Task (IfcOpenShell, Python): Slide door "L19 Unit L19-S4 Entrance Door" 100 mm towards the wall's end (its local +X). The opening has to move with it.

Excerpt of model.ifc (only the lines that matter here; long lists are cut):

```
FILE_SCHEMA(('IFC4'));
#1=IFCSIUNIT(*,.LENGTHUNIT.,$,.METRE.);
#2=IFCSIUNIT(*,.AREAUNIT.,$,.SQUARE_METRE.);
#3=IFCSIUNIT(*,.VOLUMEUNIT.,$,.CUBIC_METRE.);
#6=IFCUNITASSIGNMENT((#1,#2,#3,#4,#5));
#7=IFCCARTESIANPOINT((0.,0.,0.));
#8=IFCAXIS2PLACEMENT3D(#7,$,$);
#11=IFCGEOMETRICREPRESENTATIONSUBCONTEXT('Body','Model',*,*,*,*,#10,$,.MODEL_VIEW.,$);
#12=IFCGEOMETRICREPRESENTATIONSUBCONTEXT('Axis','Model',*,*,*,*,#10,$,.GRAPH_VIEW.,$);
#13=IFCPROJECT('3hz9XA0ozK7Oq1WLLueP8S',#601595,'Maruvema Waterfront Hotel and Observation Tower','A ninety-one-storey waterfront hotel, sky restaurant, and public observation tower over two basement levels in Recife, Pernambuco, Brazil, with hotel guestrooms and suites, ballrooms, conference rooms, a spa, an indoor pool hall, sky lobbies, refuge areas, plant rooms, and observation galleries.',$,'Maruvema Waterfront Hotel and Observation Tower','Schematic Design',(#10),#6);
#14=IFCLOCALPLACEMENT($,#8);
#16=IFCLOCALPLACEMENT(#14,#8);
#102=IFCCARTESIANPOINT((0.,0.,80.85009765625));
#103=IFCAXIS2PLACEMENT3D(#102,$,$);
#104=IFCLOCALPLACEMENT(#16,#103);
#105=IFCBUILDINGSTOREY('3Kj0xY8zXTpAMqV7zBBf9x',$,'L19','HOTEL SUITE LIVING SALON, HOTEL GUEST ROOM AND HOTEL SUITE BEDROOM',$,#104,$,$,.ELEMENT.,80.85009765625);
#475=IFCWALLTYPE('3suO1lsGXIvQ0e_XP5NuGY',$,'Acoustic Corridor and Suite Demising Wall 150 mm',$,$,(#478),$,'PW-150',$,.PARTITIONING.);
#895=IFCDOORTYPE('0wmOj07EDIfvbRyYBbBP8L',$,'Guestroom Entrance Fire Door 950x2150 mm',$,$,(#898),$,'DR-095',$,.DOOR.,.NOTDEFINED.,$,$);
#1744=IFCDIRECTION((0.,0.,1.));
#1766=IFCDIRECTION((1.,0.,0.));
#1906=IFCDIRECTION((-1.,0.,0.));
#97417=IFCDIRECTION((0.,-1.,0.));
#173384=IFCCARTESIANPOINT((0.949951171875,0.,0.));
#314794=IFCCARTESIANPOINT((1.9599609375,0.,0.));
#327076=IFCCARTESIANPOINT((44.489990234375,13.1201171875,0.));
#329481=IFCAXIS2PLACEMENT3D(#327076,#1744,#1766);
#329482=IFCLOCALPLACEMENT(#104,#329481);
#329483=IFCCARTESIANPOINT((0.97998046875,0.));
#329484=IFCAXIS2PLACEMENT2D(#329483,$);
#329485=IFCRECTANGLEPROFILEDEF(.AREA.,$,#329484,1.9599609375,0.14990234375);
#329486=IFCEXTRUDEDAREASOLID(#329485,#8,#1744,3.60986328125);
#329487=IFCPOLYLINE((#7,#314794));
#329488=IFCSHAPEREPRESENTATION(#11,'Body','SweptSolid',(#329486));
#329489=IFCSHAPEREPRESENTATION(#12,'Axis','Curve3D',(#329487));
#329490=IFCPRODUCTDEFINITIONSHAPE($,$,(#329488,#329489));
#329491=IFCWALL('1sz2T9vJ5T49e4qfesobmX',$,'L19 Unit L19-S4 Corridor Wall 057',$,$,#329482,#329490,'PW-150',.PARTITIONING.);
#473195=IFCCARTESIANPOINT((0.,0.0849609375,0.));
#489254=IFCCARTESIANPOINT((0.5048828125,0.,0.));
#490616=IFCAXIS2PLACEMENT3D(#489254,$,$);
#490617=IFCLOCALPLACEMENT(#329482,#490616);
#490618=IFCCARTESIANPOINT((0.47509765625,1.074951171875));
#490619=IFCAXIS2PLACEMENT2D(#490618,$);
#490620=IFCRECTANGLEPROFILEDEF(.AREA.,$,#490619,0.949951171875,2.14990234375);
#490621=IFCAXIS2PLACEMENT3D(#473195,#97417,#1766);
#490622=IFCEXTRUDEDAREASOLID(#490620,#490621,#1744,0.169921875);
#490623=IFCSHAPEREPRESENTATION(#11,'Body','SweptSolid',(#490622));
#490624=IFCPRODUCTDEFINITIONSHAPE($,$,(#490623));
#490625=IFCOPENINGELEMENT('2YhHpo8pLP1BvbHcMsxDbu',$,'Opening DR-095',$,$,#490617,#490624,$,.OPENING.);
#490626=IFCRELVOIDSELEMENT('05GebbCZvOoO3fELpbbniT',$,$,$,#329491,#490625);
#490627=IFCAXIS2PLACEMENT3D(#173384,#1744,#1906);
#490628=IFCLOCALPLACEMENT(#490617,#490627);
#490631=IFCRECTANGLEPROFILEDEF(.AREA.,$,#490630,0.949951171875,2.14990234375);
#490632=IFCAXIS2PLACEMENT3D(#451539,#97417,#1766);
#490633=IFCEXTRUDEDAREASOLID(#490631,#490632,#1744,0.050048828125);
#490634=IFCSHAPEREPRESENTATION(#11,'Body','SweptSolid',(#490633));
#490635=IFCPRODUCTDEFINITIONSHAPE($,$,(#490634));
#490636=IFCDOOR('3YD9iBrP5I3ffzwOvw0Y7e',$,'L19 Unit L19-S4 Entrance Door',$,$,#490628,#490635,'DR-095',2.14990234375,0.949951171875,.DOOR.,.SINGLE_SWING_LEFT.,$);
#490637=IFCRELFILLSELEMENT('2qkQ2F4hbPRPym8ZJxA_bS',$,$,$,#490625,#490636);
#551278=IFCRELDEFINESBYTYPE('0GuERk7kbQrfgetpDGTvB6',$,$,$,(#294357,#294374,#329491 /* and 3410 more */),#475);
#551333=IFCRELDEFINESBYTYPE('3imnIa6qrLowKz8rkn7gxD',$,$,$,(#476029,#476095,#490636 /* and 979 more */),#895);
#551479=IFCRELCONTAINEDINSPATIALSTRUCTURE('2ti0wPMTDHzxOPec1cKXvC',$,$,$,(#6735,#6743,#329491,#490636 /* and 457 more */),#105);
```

```python
import ifcopenshell
import ifcopenshell.api.geometry
import ifcopenshell.util.placement

model = ifcopenshell.open("model.ifc")

door = model.by_id(490636)
opening = door.FillsVoids[0].RelatingOpeningElement
wall = opening.VoidsElements[0].RelatingBuildingElement

wall_matrix = ifcopenshell.util.placement.get_local_placement(wall.ObjectPlacement)
shift = wall_matrix[:3, 0] * 0.1
before = ifcopenshell.util.placement.get_local_placement(door.ObjectPlacement)[:3, 3].copy()

# The door is placed relative to its opening, so it follows when the opening moves.
matrix = ifcopenshell.util.placement.get_local_placement(opening.ObjectPlacement)
matrix[:3, 3] += shift
ifcopenshell.api.geometry.edit_object_placement(
    model, product=opening, matrix=matrix, is_si=False, should_transform_children=True
)

after = ifcopenshell.util.placement.get_local_placement(door.ObjectPlacement)[:3, 3]
print("door moved by", (after - before).round(3) + 0.0)

model.write("model_rev.ifc")
```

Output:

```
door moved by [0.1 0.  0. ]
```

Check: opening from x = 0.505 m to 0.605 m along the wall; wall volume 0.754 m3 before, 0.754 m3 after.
